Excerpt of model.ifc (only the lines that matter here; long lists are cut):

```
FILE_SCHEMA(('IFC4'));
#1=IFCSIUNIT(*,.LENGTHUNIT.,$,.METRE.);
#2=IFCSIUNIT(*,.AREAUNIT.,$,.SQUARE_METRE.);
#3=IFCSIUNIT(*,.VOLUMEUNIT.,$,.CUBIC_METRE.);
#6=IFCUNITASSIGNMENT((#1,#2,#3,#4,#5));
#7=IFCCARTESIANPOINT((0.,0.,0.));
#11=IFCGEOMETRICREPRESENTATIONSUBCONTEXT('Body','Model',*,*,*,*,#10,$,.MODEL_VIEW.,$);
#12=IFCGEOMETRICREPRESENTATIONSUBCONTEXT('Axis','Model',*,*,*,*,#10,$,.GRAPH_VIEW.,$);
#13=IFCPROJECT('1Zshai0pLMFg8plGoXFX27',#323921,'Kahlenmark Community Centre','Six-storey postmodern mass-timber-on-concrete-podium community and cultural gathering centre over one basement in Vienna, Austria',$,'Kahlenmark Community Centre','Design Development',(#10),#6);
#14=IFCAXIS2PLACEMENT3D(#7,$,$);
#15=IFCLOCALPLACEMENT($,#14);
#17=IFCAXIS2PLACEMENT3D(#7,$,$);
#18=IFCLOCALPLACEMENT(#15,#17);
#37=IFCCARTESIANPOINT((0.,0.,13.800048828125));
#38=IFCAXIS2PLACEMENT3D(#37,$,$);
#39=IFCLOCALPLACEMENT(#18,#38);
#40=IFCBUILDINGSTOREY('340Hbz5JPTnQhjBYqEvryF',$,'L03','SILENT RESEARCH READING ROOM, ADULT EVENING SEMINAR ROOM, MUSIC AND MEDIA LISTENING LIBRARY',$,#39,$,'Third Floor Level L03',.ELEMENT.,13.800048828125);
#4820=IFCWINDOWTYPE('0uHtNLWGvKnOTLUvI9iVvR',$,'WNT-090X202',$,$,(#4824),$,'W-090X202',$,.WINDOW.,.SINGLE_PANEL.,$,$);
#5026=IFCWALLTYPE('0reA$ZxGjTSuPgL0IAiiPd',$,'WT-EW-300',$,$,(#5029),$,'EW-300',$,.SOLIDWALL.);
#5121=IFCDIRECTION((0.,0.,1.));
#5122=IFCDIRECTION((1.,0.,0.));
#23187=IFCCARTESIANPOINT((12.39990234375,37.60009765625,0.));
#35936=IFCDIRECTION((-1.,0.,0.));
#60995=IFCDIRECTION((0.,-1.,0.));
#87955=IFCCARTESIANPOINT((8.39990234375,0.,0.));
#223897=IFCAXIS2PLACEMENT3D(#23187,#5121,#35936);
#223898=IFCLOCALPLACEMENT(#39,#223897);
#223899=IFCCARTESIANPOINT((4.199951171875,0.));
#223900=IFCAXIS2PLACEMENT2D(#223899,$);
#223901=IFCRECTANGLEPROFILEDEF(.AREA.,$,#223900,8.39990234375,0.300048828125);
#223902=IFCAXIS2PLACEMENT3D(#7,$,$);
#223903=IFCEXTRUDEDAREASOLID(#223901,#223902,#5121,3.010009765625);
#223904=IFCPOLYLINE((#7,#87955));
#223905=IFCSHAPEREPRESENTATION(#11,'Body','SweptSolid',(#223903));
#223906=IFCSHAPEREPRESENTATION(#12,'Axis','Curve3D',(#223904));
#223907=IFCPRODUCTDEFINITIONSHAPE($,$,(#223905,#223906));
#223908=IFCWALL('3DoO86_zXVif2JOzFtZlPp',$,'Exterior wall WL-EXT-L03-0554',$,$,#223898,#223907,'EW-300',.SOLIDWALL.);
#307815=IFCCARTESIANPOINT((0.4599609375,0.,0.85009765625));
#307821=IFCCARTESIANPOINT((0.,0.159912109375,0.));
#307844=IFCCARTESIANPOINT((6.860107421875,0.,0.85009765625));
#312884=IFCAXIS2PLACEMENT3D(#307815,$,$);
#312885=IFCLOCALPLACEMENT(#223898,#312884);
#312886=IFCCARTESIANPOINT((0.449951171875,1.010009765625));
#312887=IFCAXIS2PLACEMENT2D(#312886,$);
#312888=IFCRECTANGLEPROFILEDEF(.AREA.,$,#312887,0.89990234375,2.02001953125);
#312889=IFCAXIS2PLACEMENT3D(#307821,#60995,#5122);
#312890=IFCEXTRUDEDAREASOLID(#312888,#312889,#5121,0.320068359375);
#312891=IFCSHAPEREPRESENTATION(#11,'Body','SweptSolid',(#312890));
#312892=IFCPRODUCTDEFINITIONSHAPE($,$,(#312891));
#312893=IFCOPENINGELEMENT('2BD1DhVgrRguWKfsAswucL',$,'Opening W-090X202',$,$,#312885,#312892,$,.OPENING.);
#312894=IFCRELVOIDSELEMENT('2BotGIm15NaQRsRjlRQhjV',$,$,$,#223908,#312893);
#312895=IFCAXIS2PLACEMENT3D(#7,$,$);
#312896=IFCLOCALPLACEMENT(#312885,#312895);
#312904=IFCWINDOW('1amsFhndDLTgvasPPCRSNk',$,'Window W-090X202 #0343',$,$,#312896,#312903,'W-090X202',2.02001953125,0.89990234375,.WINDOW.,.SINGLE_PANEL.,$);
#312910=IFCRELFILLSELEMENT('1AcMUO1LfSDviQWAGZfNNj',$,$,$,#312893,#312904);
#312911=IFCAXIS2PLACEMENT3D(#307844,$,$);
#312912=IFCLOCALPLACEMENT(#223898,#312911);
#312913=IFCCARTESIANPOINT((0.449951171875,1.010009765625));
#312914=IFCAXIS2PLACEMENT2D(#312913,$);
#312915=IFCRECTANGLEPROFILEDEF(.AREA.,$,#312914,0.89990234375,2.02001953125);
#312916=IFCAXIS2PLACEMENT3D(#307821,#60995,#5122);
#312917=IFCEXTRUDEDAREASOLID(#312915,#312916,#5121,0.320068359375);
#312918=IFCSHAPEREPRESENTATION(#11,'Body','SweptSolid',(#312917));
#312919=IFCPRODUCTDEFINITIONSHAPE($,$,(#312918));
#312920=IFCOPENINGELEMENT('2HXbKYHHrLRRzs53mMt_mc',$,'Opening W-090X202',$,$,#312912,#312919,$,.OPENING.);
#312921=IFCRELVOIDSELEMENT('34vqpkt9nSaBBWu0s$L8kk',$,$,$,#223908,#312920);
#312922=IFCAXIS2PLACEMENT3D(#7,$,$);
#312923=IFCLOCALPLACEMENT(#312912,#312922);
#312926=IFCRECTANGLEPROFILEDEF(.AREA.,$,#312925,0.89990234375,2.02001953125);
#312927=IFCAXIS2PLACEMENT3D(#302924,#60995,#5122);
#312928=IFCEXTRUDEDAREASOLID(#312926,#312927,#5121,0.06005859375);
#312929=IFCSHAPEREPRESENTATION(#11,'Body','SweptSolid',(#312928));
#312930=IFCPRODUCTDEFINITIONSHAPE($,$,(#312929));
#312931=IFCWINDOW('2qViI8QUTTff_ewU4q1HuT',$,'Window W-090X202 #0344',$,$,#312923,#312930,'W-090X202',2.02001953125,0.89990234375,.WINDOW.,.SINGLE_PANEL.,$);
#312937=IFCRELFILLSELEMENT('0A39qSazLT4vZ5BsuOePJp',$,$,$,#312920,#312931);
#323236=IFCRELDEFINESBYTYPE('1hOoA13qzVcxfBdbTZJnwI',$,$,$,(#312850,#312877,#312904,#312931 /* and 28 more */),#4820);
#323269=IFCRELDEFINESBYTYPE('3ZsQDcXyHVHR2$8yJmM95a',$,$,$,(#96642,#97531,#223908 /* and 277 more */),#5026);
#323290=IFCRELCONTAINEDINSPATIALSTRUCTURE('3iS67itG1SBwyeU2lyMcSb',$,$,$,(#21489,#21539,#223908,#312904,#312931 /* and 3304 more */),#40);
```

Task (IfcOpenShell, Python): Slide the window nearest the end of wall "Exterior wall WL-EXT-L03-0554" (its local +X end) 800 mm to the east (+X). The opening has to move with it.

```python
import ifcopenshell
import ifcopenshell.api.geometry
import ifcopenshell.util.placement

model = ifcopenshell.open("model.ifc")

window = model.by_id(312931)
opening = window.FillsVoids[0].RelatingOpeningElement
wall = opening.VoidsElements[0].RelatingBuildingElement

wall_matrix = ifcopenshell.util.placement.get_local_placement(wall.ObjectPlacement)
shift = wall_matrix[:3, 0] * -0.8
before = ifcopenshell.util.placement.get_local_placement(window.ObjectPlacement)[:3, 3].copy()

# The window is placed relative to its opening, so it follows when the opening moves.
matrix = ifcopenshell.util.placement.get_local_placement(opening.ObjectPlacement)
matrix[:3, 3] += shift
ifcopenshell.api.geometry.edit_object_placement(
    model, product=opening, matrix=matrix, is_si=False, should_transform_children=True
)

after = ifcopenshell.util.placement.get_local_placement(window.ObjectPlacement)[:3, 3]
print("window moved by", (after - before).round(3) + 0.0)

model.write("model_v2.ifc")
```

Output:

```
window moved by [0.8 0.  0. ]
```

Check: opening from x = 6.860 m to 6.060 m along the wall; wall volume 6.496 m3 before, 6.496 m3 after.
